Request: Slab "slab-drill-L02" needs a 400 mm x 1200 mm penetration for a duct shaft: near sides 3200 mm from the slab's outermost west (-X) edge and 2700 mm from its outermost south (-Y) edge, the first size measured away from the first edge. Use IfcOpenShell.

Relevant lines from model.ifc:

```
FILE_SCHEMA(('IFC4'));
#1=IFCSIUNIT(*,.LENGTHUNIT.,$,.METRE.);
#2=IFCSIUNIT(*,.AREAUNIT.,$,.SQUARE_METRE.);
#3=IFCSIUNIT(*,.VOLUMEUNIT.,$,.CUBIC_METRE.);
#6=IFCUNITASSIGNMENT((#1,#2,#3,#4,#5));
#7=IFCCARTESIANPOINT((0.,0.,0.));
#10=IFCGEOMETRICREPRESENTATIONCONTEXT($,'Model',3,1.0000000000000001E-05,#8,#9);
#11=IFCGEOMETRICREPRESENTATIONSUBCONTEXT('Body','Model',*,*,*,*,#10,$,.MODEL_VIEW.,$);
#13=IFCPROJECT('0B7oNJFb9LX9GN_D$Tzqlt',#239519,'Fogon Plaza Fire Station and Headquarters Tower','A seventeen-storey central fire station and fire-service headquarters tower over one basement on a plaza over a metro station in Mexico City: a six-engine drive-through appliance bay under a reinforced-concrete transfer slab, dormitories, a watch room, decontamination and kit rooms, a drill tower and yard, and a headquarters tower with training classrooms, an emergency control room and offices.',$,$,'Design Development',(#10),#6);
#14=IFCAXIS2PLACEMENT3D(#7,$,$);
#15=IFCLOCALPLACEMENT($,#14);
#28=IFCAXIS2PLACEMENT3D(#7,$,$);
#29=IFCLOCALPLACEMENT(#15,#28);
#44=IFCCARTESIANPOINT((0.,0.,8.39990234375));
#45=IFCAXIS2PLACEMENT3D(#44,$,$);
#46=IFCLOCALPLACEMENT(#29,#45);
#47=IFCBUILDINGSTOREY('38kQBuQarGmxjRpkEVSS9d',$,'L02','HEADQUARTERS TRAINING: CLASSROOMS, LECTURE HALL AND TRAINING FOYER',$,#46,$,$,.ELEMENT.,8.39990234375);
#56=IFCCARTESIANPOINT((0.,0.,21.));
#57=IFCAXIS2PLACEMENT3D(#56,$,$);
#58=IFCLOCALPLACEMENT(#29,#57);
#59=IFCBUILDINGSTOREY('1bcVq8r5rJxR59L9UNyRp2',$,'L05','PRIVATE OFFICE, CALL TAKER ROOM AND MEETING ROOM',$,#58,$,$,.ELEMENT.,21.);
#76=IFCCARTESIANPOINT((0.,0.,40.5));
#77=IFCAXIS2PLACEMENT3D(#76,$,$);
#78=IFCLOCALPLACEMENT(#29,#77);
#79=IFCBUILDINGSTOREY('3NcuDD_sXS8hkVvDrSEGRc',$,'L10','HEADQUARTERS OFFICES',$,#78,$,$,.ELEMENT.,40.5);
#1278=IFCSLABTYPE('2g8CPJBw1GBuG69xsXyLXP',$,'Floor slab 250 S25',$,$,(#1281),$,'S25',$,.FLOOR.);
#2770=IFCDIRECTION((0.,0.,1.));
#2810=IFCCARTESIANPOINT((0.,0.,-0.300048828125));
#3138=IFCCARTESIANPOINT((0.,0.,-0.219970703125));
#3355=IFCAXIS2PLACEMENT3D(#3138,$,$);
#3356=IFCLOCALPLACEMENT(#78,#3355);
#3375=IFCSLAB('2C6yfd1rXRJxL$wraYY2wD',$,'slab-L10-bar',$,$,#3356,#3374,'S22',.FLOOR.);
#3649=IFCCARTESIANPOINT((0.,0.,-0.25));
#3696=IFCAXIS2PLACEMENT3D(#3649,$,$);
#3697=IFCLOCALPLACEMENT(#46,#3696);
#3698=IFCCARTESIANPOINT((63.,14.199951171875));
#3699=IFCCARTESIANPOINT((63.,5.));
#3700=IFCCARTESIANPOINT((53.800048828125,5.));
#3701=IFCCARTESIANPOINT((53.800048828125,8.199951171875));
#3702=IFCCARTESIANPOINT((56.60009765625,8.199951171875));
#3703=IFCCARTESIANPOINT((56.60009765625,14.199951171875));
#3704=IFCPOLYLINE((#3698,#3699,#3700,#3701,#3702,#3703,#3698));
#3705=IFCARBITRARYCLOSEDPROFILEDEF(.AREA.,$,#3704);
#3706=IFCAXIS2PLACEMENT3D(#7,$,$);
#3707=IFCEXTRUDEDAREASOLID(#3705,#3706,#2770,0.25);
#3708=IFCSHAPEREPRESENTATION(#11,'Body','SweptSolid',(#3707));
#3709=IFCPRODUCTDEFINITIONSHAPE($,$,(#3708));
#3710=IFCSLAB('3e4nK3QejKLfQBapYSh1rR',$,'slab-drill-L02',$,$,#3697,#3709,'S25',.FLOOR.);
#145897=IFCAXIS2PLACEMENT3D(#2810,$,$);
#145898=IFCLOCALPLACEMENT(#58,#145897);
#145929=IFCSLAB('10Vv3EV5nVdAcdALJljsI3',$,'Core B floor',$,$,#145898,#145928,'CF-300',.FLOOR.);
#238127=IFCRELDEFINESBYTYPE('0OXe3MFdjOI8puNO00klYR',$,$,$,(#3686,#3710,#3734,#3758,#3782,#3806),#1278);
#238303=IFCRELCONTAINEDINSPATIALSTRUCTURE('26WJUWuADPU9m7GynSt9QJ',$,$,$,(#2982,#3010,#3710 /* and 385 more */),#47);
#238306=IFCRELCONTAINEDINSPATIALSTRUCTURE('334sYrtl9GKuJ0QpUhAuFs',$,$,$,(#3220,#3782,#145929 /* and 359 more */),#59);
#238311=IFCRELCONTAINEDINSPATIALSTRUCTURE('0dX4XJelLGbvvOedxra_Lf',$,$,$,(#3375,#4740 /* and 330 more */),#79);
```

```python
import numpy as np
import ifcopenshell
import ifcopenshell.api.feature
import ifcopenshell.api.geometry
import ifcopenshell.api.root
import ifcopenshell.geom
import ifcopenshell.util.placement
import ifcopenshell.util.representation
import ifcopenshell.util.shape
import ifcopenshell.util.unit

model = ifcopenshell.open("model.ifc")
unit_scale = ifcopenshell.util.unit.calculate_unit_scale(model)
settings = ifcopenshell.geom.settings()


def volume(element):
    """Net volume in cubic metres, openings subtracted."""
    shape = ifcopenshell.geom.create_shape(settings, element)
    return ifcopenshell.util.shape.get_volume(shape.geometry)


slab = model.by_guid("3e4nK3QejKLfQBapYSh1rR")
before = volume(slab)

# Extent in the slab's own axes, in metres. The edges named are its -X and -Y sides.
slab_shape = ifcopenshell.geom.create_shape(settings, slab)
vertices = ifcopenshell.util.shape.get_vertices(slab_shape.geometry)
x_min, y_min, bottom = vertices.min(axis=0)
top = vertices[:, 2].max()

opening = ifcopenshell.api.root.create_entity(model, ifc_class="IfcOpeningElement", name="Duct shaft opening", predefined_type="OPENING")
context = ifcopenshell.util.representation.get_context(model, "Model", "Body", "MODEL_VIEW")
width, depth = 0.4, 1.2
outline = [(0.0, 0.0), (width, 0.0), (width, depth), (0.0, depth), (0.0, 0.0)]
# Overshoot both faces by 50 mm so the cut is clean.
shape = ifcopenshell.api.geometry.add_slab_representation(
    model, context=context, depth=top - bottom + 0.1, polyline=outline
)
ifcopenshell.api.geometry.assign_representation(model, product=opening, representation=shape)

matrix = ifcopenshell.util.placement.get_local_placement(slab.ObjectPlacement)
matrix[:, 3] = matrix @ np.append(np.array([x_min + 3.2, y_min + 2.7, bottom - 0.05]) / unit_scale, 1.0)
ifcopenshell.api.geometry.edit_object_placement(model, product=opening, matrix=matrix, is_si=False)
ifcopenshell.api.feature.add_feature(model, feature=opening, element=slab)

after = volume(slab)

print(f"slab volume {before:.3f} -> {after:.3f} m3")

model.write("model_v2.ifc")
```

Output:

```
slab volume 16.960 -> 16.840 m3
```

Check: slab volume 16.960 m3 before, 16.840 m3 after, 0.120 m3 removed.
